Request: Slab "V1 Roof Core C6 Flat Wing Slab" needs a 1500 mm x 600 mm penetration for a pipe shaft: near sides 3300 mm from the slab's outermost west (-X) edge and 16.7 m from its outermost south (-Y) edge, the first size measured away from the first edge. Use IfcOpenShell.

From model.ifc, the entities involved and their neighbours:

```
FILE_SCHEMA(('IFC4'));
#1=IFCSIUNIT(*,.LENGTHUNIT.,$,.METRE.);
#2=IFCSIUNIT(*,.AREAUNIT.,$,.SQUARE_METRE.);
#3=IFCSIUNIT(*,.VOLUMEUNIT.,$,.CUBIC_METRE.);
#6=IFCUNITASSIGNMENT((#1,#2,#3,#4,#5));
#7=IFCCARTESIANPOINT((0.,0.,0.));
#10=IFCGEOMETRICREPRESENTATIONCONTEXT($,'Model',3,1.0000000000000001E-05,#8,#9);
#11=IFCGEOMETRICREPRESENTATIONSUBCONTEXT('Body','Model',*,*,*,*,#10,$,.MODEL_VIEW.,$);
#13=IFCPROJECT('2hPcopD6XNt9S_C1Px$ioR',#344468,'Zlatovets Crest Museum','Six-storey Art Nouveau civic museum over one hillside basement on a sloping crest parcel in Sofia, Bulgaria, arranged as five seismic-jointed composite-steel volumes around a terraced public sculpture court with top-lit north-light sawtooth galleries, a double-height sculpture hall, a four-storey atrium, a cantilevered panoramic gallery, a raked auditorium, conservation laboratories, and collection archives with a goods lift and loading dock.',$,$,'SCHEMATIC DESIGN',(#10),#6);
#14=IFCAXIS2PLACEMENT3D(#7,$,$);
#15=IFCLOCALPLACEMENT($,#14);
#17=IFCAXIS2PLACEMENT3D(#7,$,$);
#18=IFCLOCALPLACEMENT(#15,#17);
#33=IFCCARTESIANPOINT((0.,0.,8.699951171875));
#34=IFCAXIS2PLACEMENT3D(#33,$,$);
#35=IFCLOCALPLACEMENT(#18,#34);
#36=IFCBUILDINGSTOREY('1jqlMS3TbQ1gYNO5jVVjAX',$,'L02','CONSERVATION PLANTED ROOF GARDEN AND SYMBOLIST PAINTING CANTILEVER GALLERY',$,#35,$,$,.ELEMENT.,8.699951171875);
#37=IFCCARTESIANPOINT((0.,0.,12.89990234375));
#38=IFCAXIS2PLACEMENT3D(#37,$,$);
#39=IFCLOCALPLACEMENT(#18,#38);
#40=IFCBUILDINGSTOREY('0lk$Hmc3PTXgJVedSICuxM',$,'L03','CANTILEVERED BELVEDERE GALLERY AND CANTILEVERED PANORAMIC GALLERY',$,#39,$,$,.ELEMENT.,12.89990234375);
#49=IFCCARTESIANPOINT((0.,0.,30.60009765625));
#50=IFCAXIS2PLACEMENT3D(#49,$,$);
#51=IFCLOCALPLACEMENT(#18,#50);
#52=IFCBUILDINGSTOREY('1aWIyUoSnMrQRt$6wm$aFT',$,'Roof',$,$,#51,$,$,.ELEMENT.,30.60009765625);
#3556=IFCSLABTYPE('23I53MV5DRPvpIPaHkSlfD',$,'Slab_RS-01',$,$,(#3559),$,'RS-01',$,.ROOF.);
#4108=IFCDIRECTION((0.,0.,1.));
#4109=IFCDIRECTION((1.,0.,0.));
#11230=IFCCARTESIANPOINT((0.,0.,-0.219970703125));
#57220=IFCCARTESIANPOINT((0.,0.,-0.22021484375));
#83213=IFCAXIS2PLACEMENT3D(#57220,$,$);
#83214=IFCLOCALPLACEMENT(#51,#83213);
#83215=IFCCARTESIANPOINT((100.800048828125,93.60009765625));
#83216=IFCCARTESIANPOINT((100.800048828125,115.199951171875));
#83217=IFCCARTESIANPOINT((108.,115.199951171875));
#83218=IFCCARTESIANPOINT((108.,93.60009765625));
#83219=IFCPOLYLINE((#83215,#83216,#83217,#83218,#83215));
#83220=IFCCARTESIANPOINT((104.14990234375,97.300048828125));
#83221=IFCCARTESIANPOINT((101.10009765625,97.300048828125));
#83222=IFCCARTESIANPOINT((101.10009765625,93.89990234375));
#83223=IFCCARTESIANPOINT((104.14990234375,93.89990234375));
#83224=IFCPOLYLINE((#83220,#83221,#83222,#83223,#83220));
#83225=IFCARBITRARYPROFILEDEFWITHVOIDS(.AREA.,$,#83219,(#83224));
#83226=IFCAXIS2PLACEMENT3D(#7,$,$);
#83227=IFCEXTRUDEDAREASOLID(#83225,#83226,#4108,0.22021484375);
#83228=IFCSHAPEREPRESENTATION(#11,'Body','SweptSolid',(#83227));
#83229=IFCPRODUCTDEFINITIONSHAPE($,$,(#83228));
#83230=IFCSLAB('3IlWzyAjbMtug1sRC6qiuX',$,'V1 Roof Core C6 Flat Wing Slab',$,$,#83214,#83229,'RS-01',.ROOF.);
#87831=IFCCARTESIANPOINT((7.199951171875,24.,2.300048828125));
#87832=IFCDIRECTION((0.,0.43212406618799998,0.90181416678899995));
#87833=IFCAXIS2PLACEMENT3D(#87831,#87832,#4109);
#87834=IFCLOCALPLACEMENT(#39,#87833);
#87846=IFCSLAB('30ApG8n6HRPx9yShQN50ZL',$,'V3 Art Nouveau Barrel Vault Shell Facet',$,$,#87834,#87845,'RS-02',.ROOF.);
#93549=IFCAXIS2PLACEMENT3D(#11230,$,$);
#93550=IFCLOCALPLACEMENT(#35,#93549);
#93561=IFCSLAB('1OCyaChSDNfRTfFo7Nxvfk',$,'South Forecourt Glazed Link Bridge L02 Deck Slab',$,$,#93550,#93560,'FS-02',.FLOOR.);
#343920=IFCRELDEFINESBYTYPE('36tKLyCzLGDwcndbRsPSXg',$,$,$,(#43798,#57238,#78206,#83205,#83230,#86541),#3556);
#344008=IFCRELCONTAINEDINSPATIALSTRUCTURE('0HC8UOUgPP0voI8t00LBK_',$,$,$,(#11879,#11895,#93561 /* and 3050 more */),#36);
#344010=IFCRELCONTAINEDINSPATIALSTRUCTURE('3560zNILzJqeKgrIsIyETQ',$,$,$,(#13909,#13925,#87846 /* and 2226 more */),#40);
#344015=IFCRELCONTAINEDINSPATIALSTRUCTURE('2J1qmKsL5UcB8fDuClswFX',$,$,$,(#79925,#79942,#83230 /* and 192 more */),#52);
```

```python
import numpy as np
import ifcopenshell
import ifcopenshell.api.feature
import ifcopenshell.api.geometry
import ifcopenshell.api.root
import ifcopenshell.geom
import ifcopenshell.util.placement
import ifcopenshell.util.representation
import ifcopenshell.util.shape
import ifcopenshell.util.unit

model = ifcopenshell.open("model.ifc")
unit_scale = ifcopenshell.util.unit.calculate_unit_scale(model)
settings = ifcopenshell.geom.settings()


def volume(element):
    """Net volume in cubic metres, openings subtracted."""
    shape = ifcopenshell.geom.create_shape(settings, element)
    return ifcopenshell.util.shape.get_volume(shape.geometry)


slab = model.by_guid("3IlWzyAjbMtug1sRC6qiuX")
before = volume(slab)

# Extent in the slab's own axes, in metres. The edges named are its -X and -Y sides.
slab_shape = ifcopenshell.geom.create_shape(settings, slab)
vertices = ifcopenshell.util.shape.get_vertices(slab_shape.geometry)
x_min, y_min, bottom = vertices.min(axis=0)
top = vertices[:, 2].max()

opening = ifcopenshell.api.root.create_entity(model, ifc_class="IfcOpeningElement", name="Pipe shaft opening", predefined_type="OPENING")
context = ifcopenshell.util.representation.get_context(model, "Model", "Body", "MODEL_VIEW")
width, depth = 1.5, 0.6
outline = [(0.0, 0.0), (width, 0.0), (width, depth), (0.0, depth), (0.0, 0.0)]
# Overshoot both faces by 50 mm so the cut is clean.
shape = ifcopenshell.api.geometry.add_slab_representation(
    model, context=context, depth=top - bottom + 0.1, polyline=outline
)
ifcopenshell.api.geometry.assign_representation(model, product=opening, representation=shape)

matrix = ifcopenshell.util.placement.get_local_placement(slab.ObjectPlacement)
matrix[:, 3] = matrix @ np.append(np.array([x_min + 3.3, y_min + 16.7, bottom - 0.05]) / unit_scale, 1.0)
ifcopenshell.api.geometry.edit_object_placement(model, product=opening, matrix=matrix, is_si=False)
ifcopenshell.api.feature.add_feature(model, feature=opening, element=slab)

after = volume(slab)

print(f"slab volume {before:.3f} -> {after:.3f} m3")

model.write("model_rev.ifc")
```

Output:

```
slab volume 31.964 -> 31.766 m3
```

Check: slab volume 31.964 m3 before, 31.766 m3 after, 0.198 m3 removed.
